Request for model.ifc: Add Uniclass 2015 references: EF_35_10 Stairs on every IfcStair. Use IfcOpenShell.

First a look at what the model holds.

```python
import ifcopenshell

model = ifcopenshell.open("model.ifc")
print(model.schema)
print("classifications:", [c.Name for c in model.by_type("IfcClassification")])
for ifc_class in ("IfcDoor", "IfcRoof", "IfcStair", "IfcWall", "IfcWindow"):
    print(ifc_class, len(model.by_type(ifc_class)))
```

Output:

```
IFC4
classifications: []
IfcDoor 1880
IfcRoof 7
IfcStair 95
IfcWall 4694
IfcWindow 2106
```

```python
import ifcopenshell
import ifcopenshell.api.classification

model = ifcopenshell.open("model.ifc")

system = ifcopenshell.api.classification.add_classification(model, classification="Uniclass 2015")

codes = {
    "IfcStair": ("EF_35_10", "Stairs"),
}
for ifc_class, (code, name) in codes.items():
    products = model.by_type(ifc_class)
    ifcopenshell.api.classification.add_reference(
        model, products=products, classification=system, identification=code, name=name
    )
    print(code, len(products))

model.write("model_rev.ifc")
```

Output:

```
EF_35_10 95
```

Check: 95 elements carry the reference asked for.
